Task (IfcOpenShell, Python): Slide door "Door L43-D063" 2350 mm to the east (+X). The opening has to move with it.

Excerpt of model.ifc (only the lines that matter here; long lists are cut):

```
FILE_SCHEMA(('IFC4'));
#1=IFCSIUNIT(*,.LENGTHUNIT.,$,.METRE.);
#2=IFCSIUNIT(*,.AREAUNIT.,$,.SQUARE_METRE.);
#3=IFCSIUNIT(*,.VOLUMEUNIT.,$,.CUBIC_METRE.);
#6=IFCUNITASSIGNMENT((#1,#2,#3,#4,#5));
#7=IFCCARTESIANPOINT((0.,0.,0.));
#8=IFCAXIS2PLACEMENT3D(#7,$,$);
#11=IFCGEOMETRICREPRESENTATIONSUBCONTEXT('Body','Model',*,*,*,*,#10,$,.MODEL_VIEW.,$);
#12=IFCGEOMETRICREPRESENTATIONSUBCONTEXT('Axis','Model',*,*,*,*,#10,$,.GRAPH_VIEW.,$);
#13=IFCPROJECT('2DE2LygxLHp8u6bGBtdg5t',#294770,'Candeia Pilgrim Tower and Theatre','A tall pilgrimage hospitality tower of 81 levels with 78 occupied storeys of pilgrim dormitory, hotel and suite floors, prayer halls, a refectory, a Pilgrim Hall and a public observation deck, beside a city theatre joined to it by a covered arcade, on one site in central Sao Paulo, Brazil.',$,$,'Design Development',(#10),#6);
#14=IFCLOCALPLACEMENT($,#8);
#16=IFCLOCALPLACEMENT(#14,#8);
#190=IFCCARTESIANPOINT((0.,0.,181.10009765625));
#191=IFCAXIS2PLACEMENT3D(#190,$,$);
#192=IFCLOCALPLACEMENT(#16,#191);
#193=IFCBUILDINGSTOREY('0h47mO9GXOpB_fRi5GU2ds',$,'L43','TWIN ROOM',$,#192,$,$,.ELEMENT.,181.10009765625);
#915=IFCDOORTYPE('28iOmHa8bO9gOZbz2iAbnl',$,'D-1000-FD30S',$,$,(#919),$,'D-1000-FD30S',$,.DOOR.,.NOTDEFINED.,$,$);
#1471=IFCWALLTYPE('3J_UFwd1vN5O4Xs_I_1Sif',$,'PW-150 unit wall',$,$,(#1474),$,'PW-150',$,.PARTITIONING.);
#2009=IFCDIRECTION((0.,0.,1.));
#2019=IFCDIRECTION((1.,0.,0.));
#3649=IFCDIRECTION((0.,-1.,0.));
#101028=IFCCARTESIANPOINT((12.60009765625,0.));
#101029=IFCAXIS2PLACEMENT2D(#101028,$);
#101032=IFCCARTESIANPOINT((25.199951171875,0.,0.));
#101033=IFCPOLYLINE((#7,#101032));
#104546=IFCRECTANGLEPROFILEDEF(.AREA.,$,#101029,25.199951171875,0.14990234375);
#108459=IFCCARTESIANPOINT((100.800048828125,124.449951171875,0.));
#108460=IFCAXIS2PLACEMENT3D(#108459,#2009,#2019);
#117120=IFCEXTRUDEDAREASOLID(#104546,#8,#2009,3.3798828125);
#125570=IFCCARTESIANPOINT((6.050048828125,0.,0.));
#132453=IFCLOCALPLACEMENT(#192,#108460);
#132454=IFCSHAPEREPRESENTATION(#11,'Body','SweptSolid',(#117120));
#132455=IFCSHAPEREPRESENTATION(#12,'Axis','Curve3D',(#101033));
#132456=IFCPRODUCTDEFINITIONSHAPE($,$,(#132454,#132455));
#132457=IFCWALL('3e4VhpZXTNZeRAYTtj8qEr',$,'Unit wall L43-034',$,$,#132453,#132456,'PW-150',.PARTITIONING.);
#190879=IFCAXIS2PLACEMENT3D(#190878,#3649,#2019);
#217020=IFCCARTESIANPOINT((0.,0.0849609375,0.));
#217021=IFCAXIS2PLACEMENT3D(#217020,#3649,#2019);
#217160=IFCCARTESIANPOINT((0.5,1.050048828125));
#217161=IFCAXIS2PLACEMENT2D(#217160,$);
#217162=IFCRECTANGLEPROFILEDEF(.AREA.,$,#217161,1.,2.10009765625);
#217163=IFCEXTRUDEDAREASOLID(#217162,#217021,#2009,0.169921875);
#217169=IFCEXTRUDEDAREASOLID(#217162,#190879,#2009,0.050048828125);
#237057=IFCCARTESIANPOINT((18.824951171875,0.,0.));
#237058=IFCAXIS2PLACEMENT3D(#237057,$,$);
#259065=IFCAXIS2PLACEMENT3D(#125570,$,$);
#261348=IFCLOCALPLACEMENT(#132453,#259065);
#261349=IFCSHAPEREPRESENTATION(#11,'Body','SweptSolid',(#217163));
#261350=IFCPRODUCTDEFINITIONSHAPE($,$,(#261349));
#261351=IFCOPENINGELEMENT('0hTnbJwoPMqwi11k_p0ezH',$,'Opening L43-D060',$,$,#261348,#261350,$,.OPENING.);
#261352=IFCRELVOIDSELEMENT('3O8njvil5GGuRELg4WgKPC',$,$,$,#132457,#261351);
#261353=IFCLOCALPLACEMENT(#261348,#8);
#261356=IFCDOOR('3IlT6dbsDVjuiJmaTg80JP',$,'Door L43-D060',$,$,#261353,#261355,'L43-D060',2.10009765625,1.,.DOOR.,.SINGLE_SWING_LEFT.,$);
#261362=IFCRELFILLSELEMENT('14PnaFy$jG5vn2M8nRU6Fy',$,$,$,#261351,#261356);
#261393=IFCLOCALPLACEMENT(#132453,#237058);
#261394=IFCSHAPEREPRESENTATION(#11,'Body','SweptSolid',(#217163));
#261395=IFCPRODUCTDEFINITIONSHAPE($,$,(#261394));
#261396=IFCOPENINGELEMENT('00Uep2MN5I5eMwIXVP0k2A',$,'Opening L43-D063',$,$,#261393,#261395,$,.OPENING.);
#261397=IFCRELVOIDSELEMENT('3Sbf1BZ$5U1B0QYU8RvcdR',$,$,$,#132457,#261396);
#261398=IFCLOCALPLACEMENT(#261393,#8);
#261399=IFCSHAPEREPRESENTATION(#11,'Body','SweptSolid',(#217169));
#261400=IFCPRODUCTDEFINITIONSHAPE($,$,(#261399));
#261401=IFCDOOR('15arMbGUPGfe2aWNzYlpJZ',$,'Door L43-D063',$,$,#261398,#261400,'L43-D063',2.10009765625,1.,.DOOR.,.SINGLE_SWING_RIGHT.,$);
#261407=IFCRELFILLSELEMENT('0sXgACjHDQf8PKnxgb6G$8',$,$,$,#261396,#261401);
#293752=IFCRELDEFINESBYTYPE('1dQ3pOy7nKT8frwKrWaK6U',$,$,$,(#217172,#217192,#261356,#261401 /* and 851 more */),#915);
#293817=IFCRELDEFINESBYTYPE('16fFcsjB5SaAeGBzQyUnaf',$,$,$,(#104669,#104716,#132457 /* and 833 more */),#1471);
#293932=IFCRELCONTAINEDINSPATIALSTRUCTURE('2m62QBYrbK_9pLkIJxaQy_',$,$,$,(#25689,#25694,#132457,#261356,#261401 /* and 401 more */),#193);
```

```python
import ifcopenshell
import ifcopenshell.api.geometry
import ifcopenshell.util.placement

model = ifcopenshell.open("model.ifc")

door = model.by_id(261401)
opening = door.FillsVoids[0].RelatingOpeningElement
wall = opening.VoidsElements[0].RelatingBuildingElement

wall_matrix = ifcopenshell.util.placement.get_local_placement(wall.ObjectPlacement)
shift = wall_matrix[:3, 0] * 2.35
before = ifcopenshell.util.placement.get_local_placement(door.ObjectPlacement)[:3, 3].copy()

# The door is placed relative to its opening, so it follows when the opening moves.
matrix = ifcopenshell.util.placement.get_local_placement(opening.ObjectPlacement)
matrix[:3, 3] += shift
ifcopenshell.api.geometry.edit_object_placement(
    model, product=opening, matrix=matrix, is_si=False, should_transform_children=True
)

after = ifcopenshell.util.placement.get_local_placement(door.ObjectPlacement)[:3, 3]
print("door moved by", (after - before).round(3) + 0.0)

model.write("model_updated.ifc")
```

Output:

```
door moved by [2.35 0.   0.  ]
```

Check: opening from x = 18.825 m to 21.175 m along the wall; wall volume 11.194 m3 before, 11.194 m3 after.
